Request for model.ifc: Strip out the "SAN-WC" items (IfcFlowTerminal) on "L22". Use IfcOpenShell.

First a look at what the model holds.

```python
import ifcopenshell
import ifcopenshell.util.element

model = ifcopenshell.open("model.ifc")
print(model.schema)
storey = next(s for s in model.by_type("IfcBuildingStorey") if s.Name == "L22")
terminals = [e for e in ifcopenshell.util.element.get_decomposition(storey) if e.is_a("IfcFlowTerminal")]
seen = {}
for e in terminals:
    element_type = ifcopenshell.util.element.get_type(e)
    name = element_type.Name if element_type not in (None, e) else None
    seen[name] = seen.get(name, 0) + 1
for name, count in sorted(seen.items(), key=str):
    print(count, "x", name)
```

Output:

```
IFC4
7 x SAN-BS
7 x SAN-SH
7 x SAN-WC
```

```python
import ifcopenshell
import ifcopenshell.api.root
import ifcopenshell.util.element

model = ifcopenshell.open("model.ifc")

storey = next(s for s in model.by_type("IfcBuildingStorey") if s.Name == "L22")
terminals = [e for e in ifcopenshell.util.element.get_decomposition(storey) if e.is_a("IfcFlowTerminal")]
targets = [e for e in terminals if (t := ifcopenshell.util.element.get_type(e)) not in (None, e) and t.Name == "SAN-WC"]

for e in targets:
    ifcopenshell.api.root.remove_product(model, product=e)
print(len(targets), "removed")

model.write("model_updated.ifc")
```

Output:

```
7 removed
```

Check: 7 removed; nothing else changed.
